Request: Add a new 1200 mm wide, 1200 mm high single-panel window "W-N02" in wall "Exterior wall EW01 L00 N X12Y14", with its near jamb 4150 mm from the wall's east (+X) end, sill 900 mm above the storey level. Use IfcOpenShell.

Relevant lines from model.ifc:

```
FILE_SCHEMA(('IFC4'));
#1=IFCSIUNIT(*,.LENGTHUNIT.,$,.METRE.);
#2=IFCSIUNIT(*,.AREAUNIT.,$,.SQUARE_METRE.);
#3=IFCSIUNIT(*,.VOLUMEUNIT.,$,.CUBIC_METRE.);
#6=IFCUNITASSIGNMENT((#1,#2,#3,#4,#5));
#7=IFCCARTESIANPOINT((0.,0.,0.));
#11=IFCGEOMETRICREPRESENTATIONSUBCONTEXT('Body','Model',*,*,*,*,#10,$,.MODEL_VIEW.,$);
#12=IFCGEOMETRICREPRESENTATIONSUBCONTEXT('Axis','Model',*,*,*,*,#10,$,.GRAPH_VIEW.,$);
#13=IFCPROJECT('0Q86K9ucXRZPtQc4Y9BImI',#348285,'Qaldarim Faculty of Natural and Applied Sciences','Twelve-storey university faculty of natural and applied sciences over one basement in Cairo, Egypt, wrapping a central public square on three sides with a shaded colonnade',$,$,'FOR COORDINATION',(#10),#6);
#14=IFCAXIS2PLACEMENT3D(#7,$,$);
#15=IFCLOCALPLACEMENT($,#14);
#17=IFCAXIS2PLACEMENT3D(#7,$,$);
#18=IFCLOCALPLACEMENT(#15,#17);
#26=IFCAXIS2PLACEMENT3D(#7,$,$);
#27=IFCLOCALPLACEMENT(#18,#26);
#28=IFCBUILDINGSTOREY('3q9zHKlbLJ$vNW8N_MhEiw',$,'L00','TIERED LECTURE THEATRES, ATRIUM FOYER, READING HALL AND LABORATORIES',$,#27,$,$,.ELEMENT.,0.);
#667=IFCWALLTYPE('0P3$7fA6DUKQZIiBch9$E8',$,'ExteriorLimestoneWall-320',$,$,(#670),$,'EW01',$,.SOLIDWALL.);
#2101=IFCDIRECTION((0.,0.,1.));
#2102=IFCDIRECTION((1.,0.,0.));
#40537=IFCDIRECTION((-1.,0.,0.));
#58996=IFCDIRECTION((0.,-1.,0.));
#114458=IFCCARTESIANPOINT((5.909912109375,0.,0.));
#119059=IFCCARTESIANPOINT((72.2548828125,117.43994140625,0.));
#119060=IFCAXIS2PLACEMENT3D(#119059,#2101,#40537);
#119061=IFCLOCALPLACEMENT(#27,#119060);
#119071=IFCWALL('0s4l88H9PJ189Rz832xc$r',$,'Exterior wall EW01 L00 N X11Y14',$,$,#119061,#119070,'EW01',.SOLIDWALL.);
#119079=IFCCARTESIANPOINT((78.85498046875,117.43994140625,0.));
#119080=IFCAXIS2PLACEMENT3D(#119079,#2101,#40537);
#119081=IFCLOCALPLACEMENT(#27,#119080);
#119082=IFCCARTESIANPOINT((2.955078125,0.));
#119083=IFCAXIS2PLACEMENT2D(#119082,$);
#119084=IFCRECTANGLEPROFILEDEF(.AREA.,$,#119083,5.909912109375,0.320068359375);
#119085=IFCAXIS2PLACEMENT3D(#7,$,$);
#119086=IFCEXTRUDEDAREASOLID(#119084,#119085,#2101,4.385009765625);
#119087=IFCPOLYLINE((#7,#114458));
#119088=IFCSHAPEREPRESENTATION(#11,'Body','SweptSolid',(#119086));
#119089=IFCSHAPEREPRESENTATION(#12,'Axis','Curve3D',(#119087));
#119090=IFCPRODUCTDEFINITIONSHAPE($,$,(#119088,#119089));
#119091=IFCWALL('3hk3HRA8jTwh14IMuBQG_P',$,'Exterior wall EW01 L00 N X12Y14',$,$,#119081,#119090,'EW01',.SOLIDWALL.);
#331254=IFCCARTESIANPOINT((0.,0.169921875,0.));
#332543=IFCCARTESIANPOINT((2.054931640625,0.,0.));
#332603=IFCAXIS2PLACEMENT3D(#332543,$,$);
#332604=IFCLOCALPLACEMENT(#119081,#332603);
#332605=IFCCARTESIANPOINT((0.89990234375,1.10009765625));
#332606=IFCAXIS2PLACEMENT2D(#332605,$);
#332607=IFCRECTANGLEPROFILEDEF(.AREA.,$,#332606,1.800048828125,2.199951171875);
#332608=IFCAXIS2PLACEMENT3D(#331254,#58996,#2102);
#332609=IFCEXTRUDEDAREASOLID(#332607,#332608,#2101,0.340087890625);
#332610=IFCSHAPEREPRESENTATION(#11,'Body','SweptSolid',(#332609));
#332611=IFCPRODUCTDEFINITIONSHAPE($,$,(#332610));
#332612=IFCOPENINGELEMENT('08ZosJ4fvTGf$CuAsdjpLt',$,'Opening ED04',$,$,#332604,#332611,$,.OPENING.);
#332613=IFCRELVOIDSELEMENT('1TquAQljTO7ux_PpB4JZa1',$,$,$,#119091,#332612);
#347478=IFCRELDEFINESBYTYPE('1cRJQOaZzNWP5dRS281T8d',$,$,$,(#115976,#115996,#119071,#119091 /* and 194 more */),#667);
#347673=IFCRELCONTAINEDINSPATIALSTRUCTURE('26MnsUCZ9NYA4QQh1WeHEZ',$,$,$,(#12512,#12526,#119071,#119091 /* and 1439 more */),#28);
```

```python
import numpy as np
import ifcopenshell
import ifcopenshell.api.feature
import ifcopenshell.api.geometry
import ifcopenshell.api.root
import ifcopenshell.api.spatial
import ifcopenshell.geom
import ifcopenshell.util.element
import ifcopenshell.util.placement
import ifcopenshell.util.representation
import ifcopenshell.util.shape
import ifcopenshell.util.unit

model = ifcopenshell.open("model.ifc")
unit_scale = ifcopenshell.util.unit.calculate_unit_scale(model)
settings = ifcopenshell.geom.settings()


def volume(element):
    """Net volume in cubic metres, openings subtracted."""
    shape = ifcopenshell.geom.create_shape(settings, element)
    return ifcopenshell.util.shape.get_volume(shape.geometry)


wall = model.by_guid("3hk3HRA8jTwh14IMuBQG_P")
storey = ifcopenshell.util.element.get_container(wall, ifc_class="IfcBuildingStorey")
context = ifcopenshell.util.representation.get_context(model, "Model", "Body", "MODEL_VIEW")
before = volume(wall)

width, height, from_end, sill = 1.2, 1.2, 4.15, 0.9  # metres

# The wall runs along its own X axis, and the end named is its -X end.
wall_shape = ifcopenshell.geom.create_shape(settings, wall)
x, y, z = ifcopenshell.util.shape.get_vertices(wall_shape.geometry).T
start = x.min() + from_end
face, thickness = float(y.min()), float(y.max() - y.min())
wall_matrix = ifcopenshell.util.placement.get_local_placement(wall.ObjectPlacement)
level = ifcopenshell.util.placement.get_local_placement(storey.ObjectPlacement)[2, 3]


def in_wall(x, y):
    """Placement at x, y metres in the wall's axes, at sill height."""
    matrix = wall_matrix.copy()
    matrix[:, 3] = wall_matrix @ np.array([x / unit_scale, y / unit_scale, 0.0, 1.0])
    matrix[2, 3] = level + sill / unit_scale
    return matrix


# Opening: a box that overshoots both wall faces by 50 mm.
opening = ifcopenshell.api.root.create_entity(model, ifc_class="IfcOpeningElement", predefined_type="OPENING")
box = ifcopenshell.api.geometry.add_wall_representation(
    model, context=context, length=width, height=height, thickness=thickness + 0.1
)
ifcopenshell.api.geometry.assign_representation(model, product=opening, representation=box)
ifcopenshell.api.geometry.edit_object_placement(model, product=opening, matrix=in_wall(start, face - 0.05), is_si=False)
ifcopenshell.api.feature.add_feature(model, feature=opening, element=wall)

window = ifcopenshell.api.root.create_entity(model, ifc_class="IfcWindow", name="W-N02", predefined_type="WINDOW")
window.OverallWidth, window.OverallHeight = width / unit_scale, height / unit_scale
window.PartitioningType = "SINGLE_PANEL"
body = ifcopenshell.api.geometry.add_window_representation(
    model,
    context=context,
    overall_width=window.OverallWidth,
    overall_height=window.OverallHeight,
    partition_type="SINGLE_PANEL",
)
ifcopenshell.api.geometry.assign_representation(model, product=window, representation=body)
ifcopenshell.api.spatial.assign_container(model, products=[window], relating_structure=storey)
ifcopenshell.api.feature.add_filling(model, opening=opening, element=window)

# Centre the window in the wall's thickness.
ifcopenshell.api.geometry.edit_object_placement(model, product=window, matrix=in_wall(start, face), is_si=False)
window_shape = ifcopenshell.geom.create_shape(settings, window)
depth = ifcopenshell.util.shape.get_vertices(window_shape.geometry)[:, 1]
offset = face + thickness / 2 - (depth.min() + depth.max()) / 2
ifcopenshell.api.geometry.edit_object_placement(model, product=window, matrix=in_wall(start, offset), is_si=False)

after = volume(wall)

print(f"wall volume {before:.3f} -> {after:.3f} m3")

model.write("model-out.ifc")
```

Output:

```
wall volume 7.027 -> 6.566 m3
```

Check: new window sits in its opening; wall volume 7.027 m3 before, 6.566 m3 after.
